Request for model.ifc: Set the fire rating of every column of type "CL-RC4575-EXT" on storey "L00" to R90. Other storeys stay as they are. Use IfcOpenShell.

First a look at what the model holds.

```python
import ifcopenshell
import ifcopenshell.util.element

model = ifcopenshell.open("model.ifc")
print(model.schema)
storey = next(s for s in model.by_type("IfcBuildingStorey") if s.Name == "L00")
columns = [e for e in ifcopenshell.util.element.get_decomposition(storey) if e.is_a("IfcColumn")]
seen = {}
for e in columns:
    element_type = ifcopenshell.util.element.get_type(e)
    key = (element_type.Name if element_type != e and element_type else None, ifcopenshell.util.element.get_pset(e, "Pset_ColumnCommon", "FireRating"))
    seen[key] = seen.get(key, 0) + 1
for (name, value), count in sorted(seen.items(), key=str):
    print(count, "x", name, "|", value)
```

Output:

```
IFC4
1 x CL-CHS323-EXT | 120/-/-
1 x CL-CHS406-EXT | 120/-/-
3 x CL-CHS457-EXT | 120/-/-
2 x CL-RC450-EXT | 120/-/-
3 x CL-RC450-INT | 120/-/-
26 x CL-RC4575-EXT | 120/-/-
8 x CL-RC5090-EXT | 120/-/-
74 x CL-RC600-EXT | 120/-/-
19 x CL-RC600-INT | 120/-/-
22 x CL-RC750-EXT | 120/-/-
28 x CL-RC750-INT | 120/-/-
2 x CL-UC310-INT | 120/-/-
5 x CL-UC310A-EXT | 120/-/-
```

```python
import ifcopenshell
import ifcopenshell.api.pset
import ifcopenshell.util.element

model = ifcopenshell.open("model.ifc")

storey = next(s for s in model.by_type("IfcBuildingStorey") if s.Name == "L00")
columns = [e for e in ifcopenshell.util.element.get_decomposition(storey) if e.is_a("IfcColumn")]

count = 0
for e in columns:
    element_type = ifcopenshell.util.element.get_type(e)
    if element_type in (None, e) or element_type.Name != "CL-RC4575-EXT":
        continue
    # add_pset returns the element's existing set when there is one.
    pset = ifcopenshell.api.pset.add_pset(model, product=e, name="Pset_ColumnCommon")
    ifcopenshell.api.pset.edit_pset(model, pset=pset, properties={"FireRating": "R90"})
    count += 1

print(count, "columns updated")

model.write("model_updated.ifc")
```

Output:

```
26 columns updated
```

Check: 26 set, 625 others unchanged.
